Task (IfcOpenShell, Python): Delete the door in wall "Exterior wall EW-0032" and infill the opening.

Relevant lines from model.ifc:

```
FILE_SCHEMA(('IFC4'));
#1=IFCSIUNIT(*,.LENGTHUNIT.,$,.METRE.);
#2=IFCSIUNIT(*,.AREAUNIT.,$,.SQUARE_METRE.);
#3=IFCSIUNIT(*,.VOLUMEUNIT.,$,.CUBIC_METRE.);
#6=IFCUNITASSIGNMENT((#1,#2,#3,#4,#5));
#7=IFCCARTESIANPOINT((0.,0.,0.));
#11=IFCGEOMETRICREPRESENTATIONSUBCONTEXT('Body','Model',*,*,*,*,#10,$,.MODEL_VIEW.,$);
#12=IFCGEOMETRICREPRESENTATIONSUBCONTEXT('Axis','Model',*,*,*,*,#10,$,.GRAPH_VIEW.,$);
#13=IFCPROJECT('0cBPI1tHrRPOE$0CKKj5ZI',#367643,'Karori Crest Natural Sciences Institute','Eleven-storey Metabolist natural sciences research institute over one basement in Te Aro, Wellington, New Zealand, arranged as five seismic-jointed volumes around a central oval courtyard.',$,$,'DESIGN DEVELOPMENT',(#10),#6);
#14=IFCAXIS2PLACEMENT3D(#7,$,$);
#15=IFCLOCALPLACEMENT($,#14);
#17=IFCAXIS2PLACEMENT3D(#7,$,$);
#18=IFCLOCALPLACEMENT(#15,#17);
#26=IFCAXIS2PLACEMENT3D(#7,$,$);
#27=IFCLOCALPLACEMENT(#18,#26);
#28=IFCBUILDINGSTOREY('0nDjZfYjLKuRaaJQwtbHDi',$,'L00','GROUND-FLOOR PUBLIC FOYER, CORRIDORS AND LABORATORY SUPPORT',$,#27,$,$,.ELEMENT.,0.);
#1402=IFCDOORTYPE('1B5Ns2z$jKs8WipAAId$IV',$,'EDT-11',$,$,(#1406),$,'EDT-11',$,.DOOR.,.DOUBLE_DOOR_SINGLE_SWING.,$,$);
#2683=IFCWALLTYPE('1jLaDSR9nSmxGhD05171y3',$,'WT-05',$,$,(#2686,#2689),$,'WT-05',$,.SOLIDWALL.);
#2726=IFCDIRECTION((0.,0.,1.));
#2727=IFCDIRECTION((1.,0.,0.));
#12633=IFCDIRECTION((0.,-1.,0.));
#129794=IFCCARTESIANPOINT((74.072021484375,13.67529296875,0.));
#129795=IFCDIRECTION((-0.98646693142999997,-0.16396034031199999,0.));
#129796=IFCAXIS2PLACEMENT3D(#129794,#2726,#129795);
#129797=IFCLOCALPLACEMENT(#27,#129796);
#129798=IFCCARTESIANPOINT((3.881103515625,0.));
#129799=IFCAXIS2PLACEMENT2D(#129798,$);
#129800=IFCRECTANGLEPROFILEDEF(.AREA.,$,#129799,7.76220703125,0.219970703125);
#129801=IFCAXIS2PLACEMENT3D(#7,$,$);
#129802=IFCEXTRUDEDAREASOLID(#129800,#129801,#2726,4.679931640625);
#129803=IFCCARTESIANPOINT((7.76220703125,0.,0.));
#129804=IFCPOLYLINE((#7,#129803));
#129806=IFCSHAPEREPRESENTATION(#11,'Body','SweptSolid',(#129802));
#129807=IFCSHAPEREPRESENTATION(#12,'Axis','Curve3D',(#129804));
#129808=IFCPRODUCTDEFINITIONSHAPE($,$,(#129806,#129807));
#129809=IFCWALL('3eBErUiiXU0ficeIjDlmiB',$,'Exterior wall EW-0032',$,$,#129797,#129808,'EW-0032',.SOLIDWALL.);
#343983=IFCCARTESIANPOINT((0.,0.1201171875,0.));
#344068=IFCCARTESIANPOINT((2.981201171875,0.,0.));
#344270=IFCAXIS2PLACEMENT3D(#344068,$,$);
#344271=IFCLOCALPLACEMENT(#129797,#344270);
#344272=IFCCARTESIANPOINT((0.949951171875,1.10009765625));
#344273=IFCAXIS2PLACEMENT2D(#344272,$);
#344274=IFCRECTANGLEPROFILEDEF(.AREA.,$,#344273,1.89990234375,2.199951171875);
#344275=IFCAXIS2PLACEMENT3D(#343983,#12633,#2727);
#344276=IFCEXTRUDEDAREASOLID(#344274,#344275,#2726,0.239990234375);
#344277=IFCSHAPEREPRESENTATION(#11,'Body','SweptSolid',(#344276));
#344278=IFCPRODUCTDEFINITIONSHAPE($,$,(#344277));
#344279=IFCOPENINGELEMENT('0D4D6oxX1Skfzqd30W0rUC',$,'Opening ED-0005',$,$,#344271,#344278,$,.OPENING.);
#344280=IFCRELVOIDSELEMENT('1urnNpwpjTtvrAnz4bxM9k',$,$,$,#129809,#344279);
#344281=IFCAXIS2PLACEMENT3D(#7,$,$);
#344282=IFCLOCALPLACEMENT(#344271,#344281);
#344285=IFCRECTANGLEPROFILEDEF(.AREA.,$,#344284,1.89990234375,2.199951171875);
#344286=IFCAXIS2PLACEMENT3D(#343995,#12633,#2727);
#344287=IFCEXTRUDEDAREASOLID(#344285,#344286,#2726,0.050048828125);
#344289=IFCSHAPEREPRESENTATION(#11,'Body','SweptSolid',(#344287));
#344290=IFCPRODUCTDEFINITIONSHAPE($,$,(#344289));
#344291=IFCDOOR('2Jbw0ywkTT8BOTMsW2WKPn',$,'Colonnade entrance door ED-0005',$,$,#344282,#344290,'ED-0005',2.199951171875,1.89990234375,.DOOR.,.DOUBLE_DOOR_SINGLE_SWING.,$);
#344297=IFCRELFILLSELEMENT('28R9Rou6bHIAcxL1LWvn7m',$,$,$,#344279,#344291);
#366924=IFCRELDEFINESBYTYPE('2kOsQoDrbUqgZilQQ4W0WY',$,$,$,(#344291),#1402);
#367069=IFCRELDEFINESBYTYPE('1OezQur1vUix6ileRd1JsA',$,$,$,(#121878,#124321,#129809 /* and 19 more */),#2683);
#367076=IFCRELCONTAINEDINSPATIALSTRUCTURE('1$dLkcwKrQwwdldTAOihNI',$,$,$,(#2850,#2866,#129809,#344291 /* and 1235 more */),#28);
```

```python
import ifcopenshell
import ifcopenshell.api.feature
import ifcopenshell.api.root
import ifcopenshell.geom
import ifcopenshell.util.shape

model = ifcopenshell.open("model.ifc")
settings = ifcopenshell.geom.settings()


def volume(element):
    """Net volume in cubic metres, openings subtracted."""
    shape = ifcopenshell.geom.create_shape(settings, element)
    return ifcopenshell.util.shape.get_volume(shape.geometry)


door = model.by_guid("2Jbw0ywkTT8BOTMsW2WKPn")
opening = door.FillsVoids[0].RelatingOpeningElement
wall = opening.VoidsElements[0].RelatingBuildingElement
before = volume(wall)

ifcopenshell.api.root.remove_product(model, product=door)
ifcopenshell.api.feature.remove_feature(model, feature=opening)

after = volume(wall)

print(f"wall volume {before:.3f} -> {after:.3f} m3")

model.write("model_rev.ifc")
```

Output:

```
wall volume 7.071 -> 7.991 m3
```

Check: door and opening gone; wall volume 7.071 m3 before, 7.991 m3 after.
